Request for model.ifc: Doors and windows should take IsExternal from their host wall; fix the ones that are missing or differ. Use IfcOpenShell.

First a look at what the model holds.

```python
import ifcopenshell
import ifcopenshell.util.element

model = ifcopenshell.open("model.ifc")
print(model.schema)
seen = {}
for e in model.by_type("IfcDoor") + model.by_type("IfcWindow"):
    if not e.FillsVoids:
        continue
    host = e.FillsVoids[0].RelatingOpeningElement.VoidsElements[0].RelatingBuildingElement
    own = ifcopenshell.util.element.get_pset(e, f"Pset_{e.is_a()[3:].removesuffix('StandardCase')}Common", "IsExternal")
    wall = ifcopenshell.util.element.get_pset(host, "Pset_WallCommon", "IsExternal")
    seen[e.is_a(), own, wall] = seen.get((e.is_a(), own, wall), 0) + 1
for (cls, own, wall), count in sorted(seen.items(), key=str):
    print(count, cls, "IsExternal:", own, "| host wall:", wall)
```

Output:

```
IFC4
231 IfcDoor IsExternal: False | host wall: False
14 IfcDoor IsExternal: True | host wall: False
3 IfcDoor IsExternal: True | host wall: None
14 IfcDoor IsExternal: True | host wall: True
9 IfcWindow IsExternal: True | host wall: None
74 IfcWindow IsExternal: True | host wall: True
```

```python
import ifcopenshell
import ifcopenshell.api.pset
import ifcopenshell.util.element

model = ifcopenshell.open("model.ifc")

count = 0
for ifc_class, pset_name in (("IfcDoor", "Pset_DoorCommon"), ("IfcWindow", "Pset_WindowCommon")):
    for e in model.by_type(ifc_class):
        if not e.FillsVoids:
            continue
        host = e.FillsVoids[0].RelatingOpeningElement.VoidsElements[0].RelatingBuildingElement
        external = ifcopenshell.util.element.get_pset(host, "Pset_WallCommon", "IsExternal")
        if external is None or ifcopenshell.util.element.get_pset(e, pset_name, "IsExternal") == external:
            continue
        pset = ifcopenshell.api.pset.add_pset(model, product=e, name=pset_name)
        ifcopenshell.api.pset.edit_pset(model, pset=pset, properties={"IsExternal": external})
        count += 1

print(count, "updated")

model.write("model_updated.ifc")
```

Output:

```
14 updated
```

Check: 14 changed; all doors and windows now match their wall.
